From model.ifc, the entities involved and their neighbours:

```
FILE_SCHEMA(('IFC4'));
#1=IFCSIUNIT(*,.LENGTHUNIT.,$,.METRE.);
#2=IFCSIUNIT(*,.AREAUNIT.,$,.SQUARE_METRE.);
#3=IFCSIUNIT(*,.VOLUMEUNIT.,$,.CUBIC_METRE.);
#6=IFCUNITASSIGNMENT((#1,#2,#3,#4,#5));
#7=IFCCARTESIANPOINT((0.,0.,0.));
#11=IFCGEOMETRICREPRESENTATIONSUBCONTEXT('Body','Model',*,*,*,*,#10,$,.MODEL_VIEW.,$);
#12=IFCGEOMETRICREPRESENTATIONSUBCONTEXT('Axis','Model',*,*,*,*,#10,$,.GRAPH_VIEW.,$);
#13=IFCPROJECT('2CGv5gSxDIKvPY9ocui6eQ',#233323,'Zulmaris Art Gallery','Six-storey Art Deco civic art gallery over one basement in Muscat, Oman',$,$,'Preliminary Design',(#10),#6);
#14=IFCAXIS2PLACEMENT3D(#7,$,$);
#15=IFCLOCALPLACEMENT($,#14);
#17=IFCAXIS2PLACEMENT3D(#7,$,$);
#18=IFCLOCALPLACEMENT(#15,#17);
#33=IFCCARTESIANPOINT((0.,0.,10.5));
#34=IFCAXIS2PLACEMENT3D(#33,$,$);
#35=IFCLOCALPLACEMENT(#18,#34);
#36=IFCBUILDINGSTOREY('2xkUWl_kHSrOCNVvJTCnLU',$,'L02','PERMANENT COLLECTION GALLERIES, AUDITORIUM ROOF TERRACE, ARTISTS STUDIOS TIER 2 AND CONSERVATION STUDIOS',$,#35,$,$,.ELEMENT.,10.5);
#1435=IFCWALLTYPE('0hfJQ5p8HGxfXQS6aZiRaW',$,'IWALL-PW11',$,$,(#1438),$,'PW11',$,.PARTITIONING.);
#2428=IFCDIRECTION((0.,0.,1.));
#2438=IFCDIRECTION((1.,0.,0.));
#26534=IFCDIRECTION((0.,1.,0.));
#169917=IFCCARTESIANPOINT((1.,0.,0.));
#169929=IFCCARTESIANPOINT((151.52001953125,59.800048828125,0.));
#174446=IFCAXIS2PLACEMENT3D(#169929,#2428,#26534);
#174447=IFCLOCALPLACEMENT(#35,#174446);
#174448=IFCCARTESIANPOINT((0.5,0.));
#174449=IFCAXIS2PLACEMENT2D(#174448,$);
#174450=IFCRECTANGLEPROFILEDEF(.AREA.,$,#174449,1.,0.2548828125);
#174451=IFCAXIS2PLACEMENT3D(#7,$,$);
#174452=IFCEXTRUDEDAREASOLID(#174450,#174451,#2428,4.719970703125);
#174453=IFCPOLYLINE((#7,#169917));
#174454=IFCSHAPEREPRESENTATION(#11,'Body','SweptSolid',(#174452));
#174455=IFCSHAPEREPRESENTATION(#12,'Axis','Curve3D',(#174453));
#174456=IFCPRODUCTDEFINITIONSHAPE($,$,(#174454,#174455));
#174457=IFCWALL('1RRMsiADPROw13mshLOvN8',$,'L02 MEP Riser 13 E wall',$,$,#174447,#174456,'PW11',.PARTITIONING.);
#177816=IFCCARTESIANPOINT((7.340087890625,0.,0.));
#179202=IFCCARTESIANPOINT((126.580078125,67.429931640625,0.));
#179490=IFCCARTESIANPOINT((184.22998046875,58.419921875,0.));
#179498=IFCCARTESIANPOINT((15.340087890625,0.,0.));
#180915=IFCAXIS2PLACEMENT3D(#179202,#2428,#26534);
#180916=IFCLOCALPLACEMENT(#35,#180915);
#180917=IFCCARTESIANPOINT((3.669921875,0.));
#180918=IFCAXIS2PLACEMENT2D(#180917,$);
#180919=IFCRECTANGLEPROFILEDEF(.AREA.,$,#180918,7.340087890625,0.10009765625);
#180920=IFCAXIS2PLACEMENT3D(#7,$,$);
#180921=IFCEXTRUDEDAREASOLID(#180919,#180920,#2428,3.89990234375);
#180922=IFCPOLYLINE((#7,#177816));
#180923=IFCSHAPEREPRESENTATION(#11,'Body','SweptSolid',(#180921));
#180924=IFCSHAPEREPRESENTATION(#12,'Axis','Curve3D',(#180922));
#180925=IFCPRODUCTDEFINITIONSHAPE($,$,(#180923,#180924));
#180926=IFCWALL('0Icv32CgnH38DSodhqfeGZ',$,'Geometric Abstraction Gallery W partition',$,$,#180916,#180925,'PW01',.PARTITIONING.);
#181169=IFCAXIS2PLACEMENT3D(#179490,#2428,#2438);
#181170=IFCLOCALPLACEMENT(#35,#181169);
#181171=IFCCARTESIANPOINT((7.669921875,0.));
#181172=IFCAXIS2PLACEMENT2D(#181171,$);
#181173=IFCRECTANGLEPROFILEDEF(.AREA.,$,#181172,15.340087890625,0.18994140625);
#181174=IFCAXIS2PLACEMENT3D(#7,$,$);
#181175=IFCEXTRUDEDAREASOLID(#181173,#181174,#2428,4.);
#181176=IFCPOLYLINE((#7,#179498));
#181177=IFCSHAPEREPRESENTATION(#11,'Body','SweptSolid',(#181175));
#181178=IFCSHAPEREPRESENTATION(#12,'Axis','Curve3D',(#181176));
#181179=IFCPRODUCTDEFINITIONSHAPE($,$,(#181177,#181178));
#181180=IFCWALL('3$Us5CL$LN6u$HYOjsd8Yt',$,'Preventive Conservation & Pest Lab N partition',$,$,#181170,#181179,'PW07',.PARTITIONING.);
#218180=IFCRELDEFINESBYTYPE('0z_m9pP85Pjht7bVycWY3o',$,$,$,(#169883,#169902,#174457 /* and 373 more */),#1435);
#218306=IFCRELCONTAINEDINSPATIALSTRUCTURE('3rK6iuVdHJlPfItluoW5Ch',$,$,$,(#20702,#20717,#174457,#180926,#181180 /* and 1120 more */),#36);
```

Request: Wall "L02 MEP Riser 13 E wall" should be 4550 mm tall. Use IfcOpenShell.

```python
import ifcopenshell
import ifcopenshell.geom
import ifcopenshell.util.representation
import ifcopenshell.util.shape
import ifcopenshell.util.unit

model = ifcopenshell.open("model.ifc")
unit_scale = ifcopenshell.util.unit.calculate_unit_scale(model)
settings = ifcopenshell.geom.settings()


def volume(element):
    """Net volume in cubic metres, openings subtracted."""
    shape = ifcopenshell.geom.create_shape(settings, element)
    return ifcopenshell.util.shape.get_volume(shape.geometry)


wall = model.by_id(174457)
before = volume(wall)

body = ifcopenshell.util.representation.get_representation(wall, "Model", "Body")
solid = body.Items[0]
old_height = solid.Depth
solid.Depth = 4.55 / unit_scale
after = volume(wall)

print(f"height {old_height:g} -> {solid.Depth:g}, volume {before:.3f} -> {after:.3f} m3")

model.write("model_rev.ifc")
```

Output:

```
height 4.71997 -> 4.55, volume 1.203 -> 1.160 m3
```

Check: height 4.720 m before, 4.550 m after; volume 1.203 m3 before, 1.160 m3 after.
